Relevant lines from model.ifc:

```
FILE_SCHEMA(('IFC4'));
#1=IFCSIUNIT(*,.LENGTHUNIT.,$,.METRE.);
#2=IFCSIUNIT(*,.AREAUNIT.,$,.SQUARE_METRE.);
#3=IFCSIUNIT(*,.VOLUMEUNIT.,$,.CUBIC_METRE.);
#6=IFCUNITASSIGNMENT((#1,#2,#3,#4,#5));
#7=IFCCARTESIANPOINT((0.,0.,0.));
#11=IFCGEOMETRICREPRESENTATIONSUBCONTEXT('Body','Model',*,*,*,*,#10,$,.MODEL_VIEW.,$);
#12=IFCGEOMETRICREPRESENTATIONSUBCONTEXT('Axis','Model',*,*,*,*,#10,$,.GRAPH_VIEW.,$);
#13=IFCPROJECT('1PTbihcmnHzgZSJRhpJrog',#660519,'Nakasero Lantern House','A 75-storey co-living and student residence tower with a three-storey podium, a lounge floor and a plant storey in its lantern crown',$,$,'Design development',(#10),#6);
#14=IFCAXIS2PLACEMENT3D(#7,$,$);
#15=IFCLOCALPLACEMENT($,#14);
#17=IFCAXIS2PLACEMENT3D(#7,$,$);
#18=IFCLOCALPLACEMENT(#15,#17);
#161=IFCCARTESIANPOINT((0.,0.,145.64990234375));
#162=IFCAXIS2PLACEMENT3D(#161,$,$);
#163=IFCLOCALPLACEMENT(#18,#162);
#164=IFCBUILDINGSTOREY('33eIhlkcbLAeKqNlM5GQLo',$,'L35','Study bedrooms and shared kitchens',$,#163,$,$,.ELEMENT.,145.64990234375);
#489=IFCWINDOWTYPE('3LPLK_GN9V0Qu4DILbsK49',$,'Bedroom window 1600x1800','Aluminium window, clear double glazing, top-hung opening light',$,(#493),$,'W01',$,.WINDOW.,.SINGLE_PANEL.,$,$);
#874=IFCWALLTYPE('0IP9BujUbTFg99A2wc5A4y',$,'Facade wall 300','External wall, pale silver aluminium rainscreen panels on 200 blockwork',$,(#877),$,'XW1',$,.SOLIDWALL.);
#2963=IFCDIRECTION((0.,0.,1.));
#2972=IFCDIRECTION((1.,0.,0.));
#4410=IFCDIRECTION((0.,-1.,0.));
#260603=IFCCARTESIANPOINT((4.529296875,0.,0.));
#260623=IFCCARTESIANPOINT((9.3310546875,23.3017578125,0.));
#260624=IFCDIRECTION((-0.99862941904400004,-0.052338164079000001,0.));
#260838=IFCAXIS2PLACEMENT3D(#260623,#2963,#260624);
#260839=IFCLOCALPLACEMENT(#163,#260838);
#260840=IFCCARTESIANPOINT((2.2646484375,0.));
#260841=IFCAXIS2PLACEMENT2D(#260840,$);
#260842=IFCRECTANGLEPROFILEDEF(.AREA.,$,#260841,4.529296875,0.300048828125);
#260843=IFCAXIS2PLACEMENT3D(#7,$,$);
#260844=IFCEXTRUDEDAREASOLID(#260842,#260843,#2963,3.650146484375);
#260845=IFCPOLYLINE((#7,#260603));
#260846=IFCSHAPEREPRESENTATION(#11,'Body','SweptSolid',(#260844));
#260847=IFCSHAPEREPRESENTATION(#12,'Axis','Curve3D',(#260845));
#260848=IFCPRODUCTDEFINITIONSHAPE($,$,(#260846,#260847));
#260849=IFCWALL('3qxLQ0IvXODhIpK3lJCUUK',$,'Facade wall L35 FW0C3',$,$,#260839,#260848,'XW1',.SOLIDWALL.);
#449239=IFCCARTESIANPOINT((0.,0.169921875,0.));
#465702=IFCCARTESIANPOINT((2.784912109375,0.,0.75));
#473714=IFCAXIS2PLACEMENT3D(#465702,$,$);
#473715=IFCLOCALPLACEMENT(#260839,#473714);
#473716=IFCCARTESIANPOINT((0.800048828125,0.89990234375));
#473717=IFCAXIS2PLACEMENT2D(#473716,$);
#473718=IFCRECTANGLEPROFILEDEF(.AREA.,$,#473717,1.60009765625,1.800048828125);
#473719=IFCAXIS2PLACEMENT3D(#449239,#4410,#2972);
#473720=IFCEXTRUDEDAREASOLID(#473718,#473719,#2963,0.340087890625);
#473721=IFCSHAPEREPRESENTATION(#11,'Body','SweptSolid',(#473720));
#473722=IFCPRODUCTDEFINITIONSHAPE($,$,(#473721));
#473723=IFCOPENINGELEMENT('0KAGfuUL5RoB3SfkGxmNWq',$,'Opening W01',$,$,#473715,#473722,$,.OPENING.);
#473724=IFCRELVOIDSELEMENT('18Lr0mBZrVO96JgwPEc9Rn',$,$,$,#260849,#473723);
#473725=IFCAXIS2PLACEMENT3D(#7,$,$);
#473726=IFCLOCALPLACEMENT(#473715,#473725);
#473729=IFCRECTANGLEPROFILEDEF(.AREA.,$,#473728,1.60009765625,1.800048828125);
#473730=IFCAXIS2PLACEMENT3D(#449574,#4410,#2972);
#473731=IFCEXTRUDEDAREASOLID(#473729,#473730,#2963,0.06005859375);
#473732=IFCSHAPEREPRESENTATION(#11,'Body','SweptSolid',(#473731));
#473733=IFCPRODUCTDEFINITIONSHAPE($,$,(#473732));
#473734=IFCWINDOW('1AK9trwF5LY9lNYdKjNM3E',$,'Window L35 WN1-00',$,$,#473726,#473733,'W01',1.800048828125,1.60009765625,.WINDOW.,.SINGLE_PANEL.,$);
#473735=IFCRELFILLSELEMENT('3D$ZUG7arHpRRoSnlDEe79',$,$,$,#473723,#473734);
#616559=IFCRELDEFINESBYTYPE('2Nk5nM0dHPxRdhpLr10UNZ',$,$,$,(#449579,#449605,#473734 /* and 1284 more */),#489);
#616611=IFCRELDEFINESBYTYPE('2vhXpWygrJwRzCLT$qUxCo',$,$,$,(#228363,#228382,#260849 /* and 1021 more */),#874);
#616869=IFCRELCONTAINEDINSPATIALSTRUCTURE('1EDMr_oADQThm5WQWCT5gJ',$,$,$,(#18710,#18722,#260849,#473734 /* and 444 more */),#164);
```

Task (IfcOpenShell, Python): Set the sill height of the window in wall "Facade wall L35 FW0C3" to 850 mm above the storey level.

```python
import numpy as np
import ifcopenshell
import ifcopenshell.api.geometry
import ifcopenshell.geom
import ifcopenshell.util.element
import ifcopenshell.util.placement
import ifcopenshell.util.shape
import ifcopenshell.util.unit

model = ifcopenshell.open("model.ifc")
unit_scale = ifcopenshell.util.unit.calculate_unit_scale(model)

window = model.by_id(473734)
opening = window.FillsVoids[0].RelatingOpeningElement
storey = ifcopenshell.util.element.get_container(window, ifc_class="IfcBuildingStorey")
level = ifcopenshell.util.placement.get_local_placement(storey.ObjectPlacement)[2, 3]

# The opening's origin need not be at the sill, so measure its lowest point.
shape = ifcopenshell.geom.create_shape(ifcopenshell.geom.settings(), opening)
bottom = ifcopenshell.util.shape.get_shape_bottom_elevation(shape, shape.geometry) / unit_scale
dz = level + 0.85 - bottom

shift = np.array([0.0, 0.0, dz])
# The window is placed relative to its opening, so it follows when the opening moves.
matrix = ifcopenshell.util.placement.get_local_placement(opening.ObjectPlacement)
matrix[:3, 3] += shift
ifcopenshell.api.geometry.edit_object_placement(
    model, product=opening, matrix=matrix, is_si=False, should_transform_children=True
)

print(f"moved by {dz * unit_scale:+.3f} m")

model.write("model-out.ifc")
```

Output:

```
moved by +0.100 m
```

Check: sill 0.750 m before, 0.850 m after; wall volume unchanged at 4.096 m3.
